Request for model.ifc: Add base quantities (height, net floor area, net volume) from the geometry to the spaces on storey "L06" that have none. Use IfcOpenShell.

First a look at what the model holds.

```python
import ifcopenshell
import ifcopenshell.util.element
import ifcopenshell.util.unit

model = ifcopenshell.open("model.ifc")
print(model.schema)
for unit_type in ("LENGTHUNIT", "AREAUNIT", "VOLUMEUNIT"):
    print(unit_type, ifcopenshell.util.unit.calculate_unit_scale(model, unit_type))
storey = next(s for s in model.by_type("IfcBuildingStorey") if s.Name == "L06")
spaces = [e for e in ifcopenshell.util.element.get_decomposition(storey) if e.is_a("IfcSpace")]
for e in sorted(spaces, key=lambda e: e.id()):
    print(e.id(), e.is_a(), e.Name, list(ifcopenshell.util.element.get_psets(e, qtos_only=True)), sep=" | ")
```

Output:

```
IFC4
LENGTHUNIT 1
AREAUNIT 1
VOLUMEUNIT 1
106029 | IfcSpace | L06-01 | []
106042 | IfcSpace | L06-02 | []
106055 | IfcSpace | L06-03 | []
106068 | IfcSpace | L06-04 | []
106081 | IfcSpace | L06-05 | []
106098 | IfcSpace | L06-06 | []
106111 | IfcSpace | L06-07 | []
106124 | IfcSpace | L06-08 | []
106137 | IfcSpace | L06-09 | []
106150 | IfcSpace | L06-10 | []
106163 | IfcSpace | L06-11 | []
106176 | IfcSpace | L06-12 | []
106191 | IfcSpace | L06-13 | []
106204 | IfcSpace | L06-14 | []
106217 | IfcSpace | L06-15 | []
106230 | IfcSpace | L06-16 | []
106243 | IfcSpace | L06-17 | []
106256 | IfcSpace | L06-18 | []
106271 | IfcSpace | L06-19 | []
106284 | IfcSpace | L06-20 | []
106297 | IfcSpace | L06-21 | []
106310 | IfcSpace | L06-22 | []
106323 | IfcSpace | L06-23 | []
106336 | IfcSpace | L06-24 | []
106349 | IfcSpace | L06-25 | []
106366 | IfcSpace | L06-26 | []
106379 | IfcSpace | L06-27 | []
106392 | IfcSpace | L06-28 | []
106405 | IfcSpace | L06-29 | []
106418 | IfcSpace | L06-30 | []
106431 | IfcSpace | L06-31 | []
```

```python
import ifcopenshell
import ifcopenshell.api.pset
import ifcopenshell.geom
import ifcopenshell.util.element
import ifcopenshell.util.shape
import ifcopenshell.util.unit

model = ifcopenshell.open("model.ifc")
unit_scale = ifcopenshell.util.unit.calculate_unit_scale(model)
area_scale = ifcopenshell.util.unit.calculate_unit_scale(model, "AREAUNIT")
volume_scale = ifcopenshell.util.unit.calculate_unit_scale(model, "VOLUMEUNIT")
settings = ifcopenshell.geom.settings()

storey = next(s for s in model.by_type("IfcBuildingStorey") if s.Name == "L06")
spaces = [e for e in ifcopenshell.util.element.get_decomposition(storey) if e.is_a("IfcSpace")]

for e in sorted(spaces, key=lambda e: e.id()):
    if ifcopenshell.util.element.get_psets(e, qtos_only=True, should_inherit=False):
        continue
    # Geometry comes back in metres, in the element's own axes.
    shape = ifcopenshell.geom.create_shape(settings, e)
    values = {
        "Height": ifcopenshell.util.shape.get_z(shape.geometry) / unit_scale,
        "NetFloorArea": ifcopenshell.util.shape.get_footprint_area(shape.geometry) / area_scale,
        "NetVolume": ifcopenshell.util.shape.get_volume(shape.geometry) / volume_scale,
    }
    qto = ifcopenshell.api.pset.add_qto(model, product=e, name="Qto_SpaceBaseQuantities")
    ifcopenshell.api.pset.edit_qto(model, qto=qto, properties=values)
    print(e.id(), {k: round(v, 3) for k, v in values.items()})

model.write("model_edited.ifc")
```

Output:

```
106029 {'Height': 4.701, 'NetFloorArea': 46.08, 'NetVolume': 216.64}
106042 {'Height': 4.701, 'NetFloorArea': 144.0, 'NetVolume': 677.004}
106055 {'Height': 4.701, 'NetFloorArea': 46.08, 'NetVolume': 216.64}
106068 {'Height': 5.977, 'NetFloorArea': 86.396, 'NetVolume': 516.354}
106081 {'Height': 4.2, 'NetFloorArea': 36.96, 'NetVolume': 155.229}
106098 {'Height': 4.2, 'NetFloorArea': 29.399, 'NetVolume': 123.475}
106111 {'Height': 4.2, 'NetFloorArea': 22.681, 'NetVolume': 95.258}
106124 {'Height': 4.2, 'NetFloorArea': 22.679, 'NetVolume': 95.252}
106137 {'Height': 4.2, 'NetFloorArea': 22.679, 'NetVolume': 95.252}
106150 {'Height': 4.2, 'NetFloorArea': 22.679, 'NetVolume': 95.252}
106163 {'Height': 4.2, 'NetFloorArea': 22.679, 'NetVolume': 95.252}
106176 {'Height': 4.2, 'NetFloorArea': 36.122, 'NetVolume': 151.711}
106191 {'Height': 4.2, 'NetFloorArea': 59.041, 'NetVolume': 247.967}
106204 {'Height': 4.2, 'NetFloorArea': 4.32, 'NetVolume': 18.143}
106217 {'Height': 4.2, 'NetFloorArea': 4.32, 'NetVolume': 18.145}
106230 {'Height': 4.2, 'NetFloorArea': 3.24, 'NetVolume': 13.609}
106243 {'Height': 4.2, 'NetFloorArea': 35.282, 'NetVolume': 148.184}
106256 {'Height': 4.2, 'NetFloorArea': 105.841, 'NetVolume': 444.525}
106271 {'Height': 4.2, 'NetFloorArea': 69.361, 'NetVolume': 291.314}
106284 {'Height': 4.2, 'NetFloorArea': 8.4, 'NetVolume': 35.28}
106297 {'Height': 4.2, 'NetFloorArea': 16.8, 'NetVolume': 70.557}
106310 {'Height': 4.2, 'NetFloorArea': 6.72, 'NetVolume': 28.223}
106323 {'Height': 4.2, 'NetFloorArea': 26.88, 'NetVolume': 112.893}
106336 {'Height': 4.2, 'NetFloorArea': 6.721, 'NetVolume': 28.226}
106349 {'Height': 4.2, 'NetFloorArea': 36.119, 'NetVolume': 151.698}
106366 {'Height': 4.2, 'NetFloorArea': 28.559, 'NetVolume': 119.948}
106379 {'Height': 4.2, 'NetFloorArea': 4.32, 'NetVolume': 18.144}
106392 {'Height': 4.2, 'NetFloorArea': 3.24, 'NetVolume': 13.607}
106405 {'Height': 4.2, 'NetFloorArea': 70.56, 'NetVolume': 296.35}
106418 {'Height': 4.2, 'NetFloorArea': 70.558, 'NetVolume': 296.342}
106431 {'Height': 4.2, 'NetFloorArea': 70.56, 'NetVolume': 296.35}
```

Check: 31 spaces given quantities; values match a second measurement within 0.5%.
